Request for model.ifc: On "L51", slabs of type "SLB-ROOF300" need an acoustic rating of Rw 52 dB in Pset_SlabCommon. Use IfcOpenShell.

First a look at what the model holds.

```python
import ifcopenshell
import ifcopenshell.util.element

model = ifcopenshell.open("model.ifc")
print(model.schema)
storey = next(s for s in model.by_type("IfcBuildingStorey") if s.Name == "L51")
slabs = [e for e in ifcopenshell.util.element.get_decomposition(storey) if e.is_a("IfcSlab")]
seen = {}
for e in slabs:
    element_type = ifcopenshell.util.element.get_type(e)
    key = (element_type.Name if element_type != e and element_type else None, ifcopenshell.util.element.get_pset(e, "Pset_SlabCommon", "AcousticRating"))
    seen[key] = seen.get(key, 0) + 1
for (name, value), count in sorted(seen.items(), key=str):
    print(count, "x", name, "|", value)
```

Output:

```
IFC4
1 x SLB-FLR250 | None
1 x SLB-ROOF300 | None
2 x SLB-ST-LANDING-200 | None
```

```python
import ifcopenshell
import ifcopenshell.api.pset
import ifcopenshell.util.element

model = ifcopenshell.open("model.ifc")

storey = next(s for s in model.by_type("IfcBuildingStorey") if s.Name == "L51")
slabs = [e for e in ifcopenshell.util.element.get_decomposition(storey) if e.is_a("IfcSlab")]

count = 0
for e in slabs:
    element_type = ifcopenshell.util.element.get_type(e)
    if element_type in (None, e) or element_type.Name != "SLB-ROOF300":
        continue
    found = ifcopenshell.util.element.get_pset(e, "Pset_SlabCommon", should_inherit=False)
    if found:
        pset = model.by_id(found["id"])
        if len(ifcopenshell.util.element.get_elements_by_pset(pset)) > 1:
            pset = ifcopenshell.api.pset.unshare_pset(model, products=[e], pset=pset)[0]
    else:
        pset = ifcopenshell.api.pset.add_pset(model, product=e, name="Pset_SlabCommon")
    ifcopenshell.api.pset.edit_pset(model, pset=pset, properties={"AcousticRating": "Rw 52 dB"})
    count += 1

print(count, "slabs updated")

model.write("model_rev.ifc")
```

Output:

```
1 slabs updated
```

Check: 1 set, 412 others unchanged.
